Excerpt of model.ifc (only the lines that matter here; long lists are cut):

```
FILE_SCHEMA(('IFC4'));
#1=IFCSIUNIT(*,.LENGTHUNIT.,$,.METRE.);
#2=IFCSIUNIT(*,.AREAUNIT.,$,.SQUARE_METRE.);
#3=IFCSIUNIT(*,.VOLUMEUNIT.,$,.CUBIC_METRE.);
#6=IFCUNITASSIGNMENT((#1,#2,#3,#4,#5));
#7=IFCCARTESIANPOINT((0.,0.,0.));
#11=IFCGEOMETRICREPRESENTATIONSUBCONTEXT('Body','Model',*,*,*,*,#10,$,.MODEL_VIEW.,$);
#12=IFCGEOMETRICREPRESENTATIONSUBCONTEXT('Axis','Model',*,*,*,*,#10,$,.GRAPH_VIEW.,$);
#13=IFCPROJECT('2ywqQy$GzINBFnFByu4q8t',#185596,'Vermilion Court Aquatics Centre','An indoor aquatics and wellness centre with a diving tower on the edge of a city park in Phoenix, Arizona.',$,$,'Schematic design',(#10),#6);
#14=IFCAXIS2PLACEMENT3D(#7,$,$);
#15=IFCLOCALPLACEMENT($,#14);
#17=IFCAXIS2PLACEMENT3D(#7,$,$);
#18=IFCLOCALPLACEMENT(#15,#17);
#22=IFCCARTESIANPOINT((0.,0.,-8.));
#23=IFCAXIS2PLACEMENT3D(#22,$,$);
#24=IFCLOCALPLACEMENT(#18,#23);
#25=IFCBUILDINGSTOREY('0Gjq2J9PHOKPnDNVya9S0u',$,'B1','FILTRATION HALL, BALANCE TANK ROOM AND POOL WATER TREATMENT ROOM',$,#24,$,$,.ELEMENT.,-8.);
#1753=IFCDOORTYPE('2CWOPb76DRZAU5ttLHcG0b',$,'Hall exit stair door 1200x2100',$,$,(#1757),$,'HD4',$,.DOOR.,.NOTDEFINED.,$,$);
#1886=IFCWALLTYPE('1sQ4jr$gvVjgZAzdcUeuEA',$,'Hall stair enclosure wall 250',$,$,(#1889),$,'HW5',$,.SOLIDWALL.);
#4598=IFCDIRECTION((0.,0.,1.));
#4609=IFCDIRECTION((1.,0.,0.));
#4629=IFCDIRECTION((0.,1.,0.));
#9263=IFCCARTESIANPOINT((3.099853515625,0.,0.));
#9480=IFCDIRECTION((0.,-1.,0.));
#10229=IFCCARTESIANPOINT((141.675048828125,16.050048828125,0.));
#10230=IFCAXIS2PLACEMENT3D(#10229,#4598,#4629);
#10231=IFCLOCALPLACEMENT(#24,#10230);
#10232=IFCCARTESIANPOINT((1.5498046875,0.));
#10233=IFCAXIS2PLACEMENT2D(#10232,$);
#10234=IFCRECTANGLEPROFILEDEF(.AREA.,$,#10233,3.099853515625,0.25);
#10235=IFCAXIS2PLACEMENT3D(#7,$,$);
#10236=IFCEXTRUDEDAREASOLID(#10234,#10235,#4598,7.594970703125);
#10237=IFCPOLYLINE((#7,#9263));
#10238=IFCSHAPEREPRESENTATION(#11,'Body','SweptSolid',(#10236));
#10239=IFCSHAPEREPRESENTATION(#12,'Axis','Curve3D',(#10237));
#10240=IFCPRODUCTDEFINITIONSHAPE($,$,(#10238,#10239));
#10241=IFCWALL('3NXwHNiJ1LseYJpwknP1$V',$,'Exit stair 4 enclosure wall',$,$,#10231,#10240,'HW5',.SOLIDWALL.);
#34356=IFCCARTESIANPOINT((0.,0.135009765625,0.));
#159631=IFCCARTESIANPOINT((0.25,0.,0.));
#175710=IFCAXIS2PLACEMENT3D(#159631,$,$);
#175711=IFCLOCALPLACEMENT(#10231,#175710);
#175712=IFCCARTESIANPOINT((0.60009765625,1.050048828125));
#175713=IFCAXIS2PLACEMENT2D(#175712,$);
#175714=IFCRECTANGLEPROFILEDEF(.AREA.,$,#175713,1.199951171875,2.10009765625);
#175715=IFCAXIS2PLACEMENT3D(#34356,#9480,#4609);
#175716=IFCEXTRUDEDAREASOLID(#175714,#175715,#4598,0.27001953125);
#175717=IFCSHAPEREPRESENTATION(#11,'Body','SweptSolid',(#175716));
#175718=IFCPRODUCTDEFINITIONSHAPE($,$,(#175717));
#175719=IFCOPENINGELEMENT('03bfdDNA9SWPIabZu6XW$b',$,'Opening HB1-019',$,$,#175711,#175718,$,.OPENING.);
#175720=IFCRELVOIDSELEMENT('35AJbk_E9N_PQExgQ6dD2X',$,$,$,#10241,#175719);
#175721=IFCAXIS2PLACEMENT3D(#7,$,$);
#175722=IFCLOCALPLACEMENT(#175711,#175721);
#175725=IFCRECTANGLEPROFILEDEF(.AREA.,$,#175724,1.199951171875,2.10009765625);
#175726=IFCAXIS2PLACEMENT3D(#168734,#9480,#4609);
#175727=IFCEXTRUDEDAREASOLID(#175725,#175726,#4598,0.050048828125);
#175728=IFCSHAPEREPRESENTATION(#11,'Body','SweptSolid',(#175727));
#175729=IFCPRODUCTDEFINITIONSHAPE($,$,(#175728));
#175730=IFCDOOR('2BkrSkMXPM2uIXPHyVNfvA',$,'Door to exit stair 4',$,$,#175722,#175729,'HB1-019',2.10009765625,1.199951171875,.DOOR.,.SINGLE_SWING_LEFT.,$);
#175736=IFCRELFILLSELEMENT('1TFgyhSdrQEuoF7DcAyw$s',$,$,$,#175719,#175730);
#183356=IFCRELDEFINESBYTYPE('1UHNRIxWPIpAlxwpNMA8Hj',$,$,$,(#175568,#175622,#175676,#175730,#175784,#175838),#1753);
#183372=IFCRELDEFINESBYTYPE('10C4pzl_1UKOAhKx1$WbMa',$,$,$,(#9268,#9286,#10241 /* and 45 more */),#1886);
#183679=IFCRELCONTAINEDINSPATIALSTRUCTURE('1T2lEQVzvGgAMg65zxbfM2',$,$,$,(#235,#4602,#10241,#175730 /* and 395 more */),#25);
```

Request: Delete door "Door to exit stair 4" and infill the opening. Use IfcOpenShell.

```python
import ifcopenshell
import ifcopenshell.api.feature
import ifcopenshell.api.root
import ifcopenshell.geom
import ifcopenshell.util.shape

model = ifcopenshell.open("model.ifc")
settings = ifcopenshell.geom.settings()


def volume(element):
    """Net volume in cubic metres, openings subtracted."""
    shape = ifcopenshell.geom.create_shape(settings, element)
    return ifcopenshell.util.shape.get_volume(shape.geometry)


door = model.by_guid("2BkrSkMXPM2uIXPHyVNfvA")
opening = door.FillsVoids[0].RelatingOpeningElement
wall = opening.VoidsElements[0].RelatingBuildingElement
before = volume(wall)

ifcopenshell.api.root.remove_product(model, product=door)
ifcopenshell.api.feature.remove_feature(model, feature=opening)

after = volume(wall)

print(f"wall volume {before:.3f} -> {after:.3f} m3")

model.write("model_rev.ifc")
```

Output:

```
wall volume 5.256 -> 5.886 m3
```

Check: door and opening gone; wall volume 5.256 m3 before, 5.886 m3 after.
